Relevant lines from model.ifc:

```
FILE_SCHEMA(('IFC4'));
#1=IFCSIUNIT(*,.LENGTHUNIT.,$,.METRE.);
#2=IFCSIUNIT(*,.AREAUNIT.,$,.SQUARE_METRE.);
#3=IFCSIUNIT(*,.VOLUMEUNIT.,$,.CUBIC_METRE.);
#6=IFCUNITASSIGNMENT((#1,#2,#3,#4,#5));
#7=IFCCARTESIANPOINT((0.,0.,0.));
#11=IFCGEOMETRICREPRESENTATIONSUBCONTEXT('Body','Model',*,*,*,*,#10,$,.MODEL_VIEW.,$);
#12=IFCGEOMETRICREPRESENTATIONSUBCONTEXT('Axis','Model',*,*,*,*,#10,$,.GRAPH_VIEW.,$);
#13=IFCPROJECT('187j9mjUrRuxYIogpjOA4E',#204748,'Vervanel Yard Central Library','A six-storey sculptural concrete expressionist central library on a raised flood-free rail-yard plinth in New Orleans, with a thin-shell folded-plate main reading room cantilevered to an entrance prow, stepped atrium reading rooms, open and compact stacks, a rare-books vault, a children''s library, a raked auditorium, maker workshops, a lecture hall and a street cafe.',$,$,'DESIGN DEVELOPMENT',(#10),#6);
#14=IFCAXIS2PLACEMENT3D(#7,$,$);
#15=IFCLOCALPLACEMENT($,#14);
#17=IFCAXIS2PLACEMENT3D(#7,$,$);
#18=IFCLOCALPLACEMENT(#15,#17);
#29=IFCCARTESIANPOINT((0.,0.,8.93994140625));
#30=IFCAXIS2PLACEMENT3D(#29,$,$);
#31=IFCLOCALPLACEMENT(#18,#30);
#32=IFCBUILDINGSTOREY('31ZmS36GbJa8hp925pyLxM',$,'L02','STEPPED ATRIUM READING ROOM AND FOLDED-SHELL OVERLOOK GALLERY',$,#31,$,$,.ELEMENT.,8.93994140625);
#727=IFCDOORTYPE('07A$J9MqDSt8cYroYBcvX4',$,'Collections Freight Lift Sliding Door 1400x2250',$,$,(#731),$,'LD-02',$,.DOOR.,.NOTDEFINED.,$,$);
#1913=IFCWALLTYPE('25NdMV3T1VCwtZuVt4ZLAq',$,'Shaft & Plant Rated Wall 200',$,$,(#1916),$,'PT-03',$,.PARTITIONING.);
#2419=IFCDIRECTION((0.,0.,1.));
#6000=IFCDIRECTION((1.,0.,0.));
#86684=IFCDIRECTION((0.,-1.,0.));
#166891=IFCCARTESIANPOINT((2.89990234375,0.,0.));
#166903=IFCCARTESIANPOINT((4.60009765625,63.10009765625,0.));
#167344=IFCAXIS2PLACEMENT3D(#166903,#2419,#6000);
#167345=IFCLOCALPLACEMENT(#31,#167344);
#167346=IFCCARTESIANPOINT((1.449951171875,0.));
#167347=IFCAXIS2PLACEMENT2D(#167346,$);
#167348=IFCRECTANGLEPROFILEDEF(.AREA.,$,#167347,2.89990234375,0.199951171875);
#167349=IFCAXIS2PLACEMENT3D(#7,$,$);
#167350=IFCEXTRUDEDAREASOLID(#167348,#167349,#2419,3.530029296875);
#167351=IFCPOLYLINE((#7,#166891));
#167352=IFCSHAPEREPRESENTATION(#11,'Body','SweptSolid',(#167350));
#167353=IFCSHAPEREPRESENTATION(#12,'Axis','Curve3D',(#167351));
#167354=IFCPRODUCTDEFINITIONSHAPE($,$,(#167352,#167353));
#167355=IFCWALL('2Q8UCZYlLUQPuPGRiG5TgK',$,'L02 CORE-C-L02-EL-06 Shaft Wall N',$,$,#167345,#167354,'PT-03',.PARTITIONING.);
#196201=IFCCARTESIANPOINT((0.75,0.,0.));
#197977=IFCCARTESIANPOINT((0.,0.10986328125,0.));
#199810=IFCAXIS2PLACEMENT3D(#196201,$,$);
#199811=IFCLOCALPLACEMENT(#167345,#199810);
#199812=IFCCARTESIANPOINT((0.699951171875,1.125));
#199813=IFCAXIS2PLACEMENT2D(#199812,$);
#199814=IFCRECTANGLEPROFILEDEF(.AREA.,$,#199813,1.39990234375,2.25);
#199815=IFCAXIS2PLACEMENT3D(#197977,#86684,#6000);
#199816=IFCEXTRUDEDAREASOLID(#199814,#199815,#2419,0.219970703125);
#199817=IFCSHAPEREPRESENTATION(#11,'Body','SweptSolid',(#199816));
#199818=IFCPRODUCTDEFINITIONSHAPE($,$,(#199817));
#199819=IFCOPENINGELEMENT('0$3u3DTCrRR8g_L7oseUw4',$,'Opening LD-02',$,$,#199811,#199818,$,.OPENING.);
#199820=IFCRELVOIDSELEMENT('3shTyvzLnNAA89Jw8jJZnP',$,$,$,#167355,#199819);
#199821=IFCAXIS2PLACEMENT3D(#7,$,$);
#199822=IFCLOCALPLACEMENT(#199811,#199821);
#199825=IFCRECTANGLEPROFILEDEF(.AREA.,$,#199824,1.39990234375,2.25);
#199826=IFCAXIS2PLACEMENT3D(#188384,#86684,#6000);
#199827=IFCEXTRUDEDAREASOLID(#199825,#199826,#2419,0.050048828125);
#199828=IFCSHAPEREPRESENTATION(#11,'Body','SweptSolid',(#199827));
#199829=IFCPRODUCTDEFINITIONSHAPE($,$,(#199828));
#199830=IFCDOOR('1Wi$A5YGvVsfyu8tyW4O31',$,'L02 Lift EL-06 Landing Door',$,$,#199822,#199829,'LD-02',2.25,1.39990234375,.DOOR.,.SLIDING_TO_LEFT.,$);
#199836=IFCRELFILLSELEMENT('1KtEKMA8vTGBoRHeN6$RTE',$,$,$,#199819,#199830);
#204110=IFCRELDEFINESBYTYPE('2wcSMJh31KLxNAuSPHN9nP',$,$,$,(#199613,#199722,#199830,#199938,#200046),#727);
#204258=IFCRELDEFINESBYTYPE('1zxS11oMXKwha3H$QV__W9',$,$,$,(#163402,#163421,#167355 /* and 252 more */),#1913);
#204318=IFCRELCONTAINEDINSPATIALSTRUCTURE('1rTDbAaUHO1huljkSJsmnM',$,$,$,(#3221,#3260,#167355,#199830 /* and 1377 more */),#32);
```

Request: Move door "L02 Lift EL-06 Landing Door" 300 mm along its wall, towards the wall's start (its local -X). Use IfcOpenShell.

```python
import ifcopenshell
import ifcopenshell.api.geometry
import ifcopenshell.util.placement
import ifcopenshell.util.unit

model = ifcopenshell.open("model.ifc")
unit_scale = ifcopenshell.util.unit.calculate_unit_scale(model)

door = model.by_guid("1Wi$A5YGvVsfyu8tyW4O31")
opening = door.FillsVoids[0].RelatingOpeningElement
wall = opening.VoidsElements[0].RelatingBuildingElement

wall_matrix = ifcopenshell.util.placement.get_local_placement(wall.ObjectPlacement)
shift = wall_matrix[:3, 0] * -0.3 / unit_scale
before = ifcopenshell.util.placement.get_local_placement(door.ObjectPlacement)[:3, 3].copy()

# The door is placed relative to its opening, so it follows when the opening moves.
matrix = ifcopenshell.util.placement.get_local_placement(opening.ObjectPlacement)
matrix[:3, 3] += shift
ifcopenshell.api.geometry.edit_object_placement(
    model, product=opening, matrix=matrix, is_si=False, should_transform_children=True
)

after = ifcopenshell.util.placement.get_local_placement(door.ObjectPlacement)[:3, 3]
print("door moved by", (after - before).round(3) + 0.0)

model.write("model_rev.ifc")
```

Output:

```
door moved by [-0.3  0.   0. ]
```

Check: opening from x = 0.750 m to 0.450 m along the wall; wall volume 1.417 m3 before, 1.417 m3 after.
